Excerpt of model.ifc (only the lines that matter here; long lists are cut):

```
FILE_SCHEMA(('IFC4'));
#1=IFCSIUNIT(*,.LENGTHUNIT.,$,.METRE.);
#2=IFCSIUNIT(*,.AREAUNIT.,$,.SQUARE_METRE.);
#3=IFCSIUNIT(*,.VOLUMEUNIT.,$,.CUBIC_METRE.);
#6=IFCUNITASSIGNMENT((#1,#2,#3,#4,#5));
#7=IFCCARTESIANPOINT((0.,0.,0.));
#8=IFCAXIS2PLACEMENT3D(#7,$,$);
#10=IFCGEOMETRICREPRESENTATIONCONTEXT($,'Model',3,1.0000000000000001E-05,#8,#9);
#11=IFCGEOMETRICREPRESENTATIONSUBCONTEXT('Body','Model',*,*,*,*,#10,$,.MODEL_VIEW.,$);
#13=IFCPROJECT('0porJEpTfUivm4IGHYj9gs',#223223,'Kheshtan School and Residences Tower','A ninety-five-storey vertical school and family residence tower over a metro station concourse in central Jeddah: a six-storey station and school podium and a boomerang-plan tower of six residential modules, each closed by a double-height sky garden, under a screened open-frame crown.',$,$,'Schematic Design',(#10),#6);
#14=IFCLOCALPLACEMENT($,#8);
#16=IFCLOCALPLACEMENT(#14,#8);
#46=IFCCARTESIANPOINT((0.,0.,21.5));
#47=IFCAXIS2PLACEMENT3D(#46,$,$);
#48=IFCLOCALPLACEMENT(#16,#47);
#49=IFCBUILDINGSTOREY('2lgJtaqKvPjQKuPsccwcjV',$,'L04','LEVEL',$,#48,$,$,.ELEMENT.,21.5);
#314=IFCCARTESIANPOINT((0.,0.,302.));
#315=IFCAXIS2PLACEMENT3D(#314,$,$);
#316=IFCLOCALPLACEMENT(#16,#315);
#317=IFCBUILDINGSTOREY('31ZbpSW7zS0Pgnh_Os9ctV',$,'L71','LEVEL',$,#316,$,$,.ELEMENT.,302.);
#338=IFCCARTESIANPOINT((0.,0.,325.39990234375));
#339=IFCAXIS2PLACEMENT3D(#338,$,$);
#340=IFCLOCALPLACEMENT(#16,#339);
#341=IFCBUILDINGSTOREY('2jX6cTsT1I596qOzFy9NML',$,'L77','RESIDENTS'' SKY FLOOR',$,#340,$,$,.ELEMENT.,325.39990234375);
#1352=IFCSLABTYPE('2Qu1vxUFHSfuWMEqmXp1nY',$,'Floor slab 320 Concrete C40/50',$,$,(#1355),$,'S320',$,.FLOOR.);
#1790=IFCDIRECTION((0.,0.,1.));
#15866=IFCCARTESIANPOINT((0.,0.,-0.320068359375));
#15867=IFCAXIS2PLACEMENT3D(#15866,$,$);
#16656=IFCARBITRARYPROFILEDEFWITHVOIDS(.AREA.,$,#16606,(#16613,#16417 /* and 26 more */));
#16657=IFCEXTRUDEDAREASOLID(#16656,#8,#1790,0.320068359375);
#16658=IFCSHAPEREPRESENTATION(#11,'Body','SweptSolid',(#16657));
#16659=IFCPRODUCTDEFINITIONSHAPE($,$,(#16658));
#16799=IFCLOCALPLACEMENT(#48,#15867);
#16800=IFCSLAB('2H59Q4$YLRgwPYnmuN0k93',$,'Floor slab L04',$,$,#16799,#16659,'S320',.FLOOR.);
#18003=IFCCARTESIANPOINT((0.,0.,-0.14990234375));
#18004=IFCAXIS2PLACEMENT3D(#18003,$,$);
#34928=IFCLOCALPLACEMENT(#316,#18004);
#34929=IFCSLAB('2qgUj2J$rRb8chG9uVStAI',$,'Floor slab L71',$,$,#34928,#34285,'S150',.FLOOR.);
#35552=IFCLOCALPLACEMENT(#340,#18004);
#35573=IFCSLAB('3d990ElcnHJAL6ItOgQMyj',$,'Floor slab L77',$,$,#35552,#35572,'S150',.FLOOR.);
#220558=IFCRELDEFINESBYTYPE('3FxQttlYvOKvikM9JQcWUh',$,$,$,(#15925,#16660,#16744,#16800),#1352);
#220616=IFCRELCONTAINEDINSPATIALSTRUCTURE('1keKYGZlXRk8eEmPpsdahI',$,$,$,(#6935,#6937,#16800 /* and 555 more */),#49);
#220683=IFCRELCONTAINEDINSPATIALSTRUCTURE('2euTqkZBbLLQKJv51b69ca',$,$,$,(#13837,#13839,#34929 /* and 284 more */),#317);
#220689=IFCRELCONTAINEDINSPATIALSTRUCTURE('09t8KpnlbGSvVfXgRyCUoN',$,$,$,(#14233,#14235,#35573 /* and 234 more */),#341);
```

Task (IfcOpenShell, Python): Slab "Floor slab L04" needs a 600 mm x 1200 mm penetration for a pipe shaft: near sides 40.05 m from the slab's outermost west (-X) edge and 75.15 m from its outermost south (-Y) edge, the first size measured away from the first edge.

```python
import numpy as np
import ifcopenshell
import ifcopenshell.api.feature
import ifcopenshell.api.geometry
import ifcopenshell.api.root
import ifcopenshell.geom
import ifcopenshell.util.placement
import ifcopenshell.util.representation
import ifcopenshell.util.shape
import ifcopenshell.util.unit

model = ifcopenshell.open("model.ifc")
unit_scale = ifcopenshell.util.unit.calculate_unit_scale(model)
settings = ifcopenshell.geom.settings()


def volume(element):
    """Net volume in cubic metres, openings subtracted."""
    shape = ifcopenshell.geom.create_shape(settings, element)
    return ifcopenshell.util.shape.get_volume(shape.geometry)


slab = model.by_guid("2H59Q4$YLRgwPYnmuN0k93")
before = volume(slab)

# Extent in the slab's own axes, in metres. The edges named are its -X and -Y sides.
slab_shape = ifcopenshell.geom.create_shape(settings, slab)
vertices = ifcopenshell.util.shape.get_vertices(slab_shape.geometry)
x_min, y_min, bottom = vertices.min(axis=0)
top = vertices[:, 2].max()

opening = ifcopenshell.api.root.create_entity(model, ifc_class="IfcOpeningElement", name="Pipe shaft opening", predefined_type="OPENING")
context = ifcopenshell.util.representation.get_context(model, "Model", "Body", "MODEL_VIEW")
width, depth = 0.6, 1.2
outline = [(0.0, 0.0), (width, 0.0), (width, depth), (0.0, depth), (0.0, 0.0)]
# Overshoot both faces by 50 mm so the cut is clean.
shape = ifcopenshell.api.geometry.add_slab_representation(
    model, context=context, depth=top - bottom + 0.1, polyline=outline
)
ifcopenshell.api.geometry.assign_representation(model, product=opening, representation=shape)

matrix = ifcopenshell.util.placement.get_local_placement(slab.ObjectPlacement)
matrix[:, 3] = matrix @ np.append(np.array([x_min + 40.05, y_min + 75.15, bottom - 0.05]) / unit_scale, 1.0)
ifcopenshell.api.geometry.edit_object_placement(model, product=opening, matrix=matrix, is_si=False)
ifcopenshell.api.feature.add_feature(model, feature=opening, element=slab)

after = volume(slab)

print(f"slab volume {before:.3f} -> {after:.3f} m3")

model.write("model-out.ifc")
```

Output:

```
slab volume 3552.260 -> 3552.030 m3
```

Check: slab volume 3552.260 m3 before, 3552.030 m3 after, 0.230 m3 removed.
